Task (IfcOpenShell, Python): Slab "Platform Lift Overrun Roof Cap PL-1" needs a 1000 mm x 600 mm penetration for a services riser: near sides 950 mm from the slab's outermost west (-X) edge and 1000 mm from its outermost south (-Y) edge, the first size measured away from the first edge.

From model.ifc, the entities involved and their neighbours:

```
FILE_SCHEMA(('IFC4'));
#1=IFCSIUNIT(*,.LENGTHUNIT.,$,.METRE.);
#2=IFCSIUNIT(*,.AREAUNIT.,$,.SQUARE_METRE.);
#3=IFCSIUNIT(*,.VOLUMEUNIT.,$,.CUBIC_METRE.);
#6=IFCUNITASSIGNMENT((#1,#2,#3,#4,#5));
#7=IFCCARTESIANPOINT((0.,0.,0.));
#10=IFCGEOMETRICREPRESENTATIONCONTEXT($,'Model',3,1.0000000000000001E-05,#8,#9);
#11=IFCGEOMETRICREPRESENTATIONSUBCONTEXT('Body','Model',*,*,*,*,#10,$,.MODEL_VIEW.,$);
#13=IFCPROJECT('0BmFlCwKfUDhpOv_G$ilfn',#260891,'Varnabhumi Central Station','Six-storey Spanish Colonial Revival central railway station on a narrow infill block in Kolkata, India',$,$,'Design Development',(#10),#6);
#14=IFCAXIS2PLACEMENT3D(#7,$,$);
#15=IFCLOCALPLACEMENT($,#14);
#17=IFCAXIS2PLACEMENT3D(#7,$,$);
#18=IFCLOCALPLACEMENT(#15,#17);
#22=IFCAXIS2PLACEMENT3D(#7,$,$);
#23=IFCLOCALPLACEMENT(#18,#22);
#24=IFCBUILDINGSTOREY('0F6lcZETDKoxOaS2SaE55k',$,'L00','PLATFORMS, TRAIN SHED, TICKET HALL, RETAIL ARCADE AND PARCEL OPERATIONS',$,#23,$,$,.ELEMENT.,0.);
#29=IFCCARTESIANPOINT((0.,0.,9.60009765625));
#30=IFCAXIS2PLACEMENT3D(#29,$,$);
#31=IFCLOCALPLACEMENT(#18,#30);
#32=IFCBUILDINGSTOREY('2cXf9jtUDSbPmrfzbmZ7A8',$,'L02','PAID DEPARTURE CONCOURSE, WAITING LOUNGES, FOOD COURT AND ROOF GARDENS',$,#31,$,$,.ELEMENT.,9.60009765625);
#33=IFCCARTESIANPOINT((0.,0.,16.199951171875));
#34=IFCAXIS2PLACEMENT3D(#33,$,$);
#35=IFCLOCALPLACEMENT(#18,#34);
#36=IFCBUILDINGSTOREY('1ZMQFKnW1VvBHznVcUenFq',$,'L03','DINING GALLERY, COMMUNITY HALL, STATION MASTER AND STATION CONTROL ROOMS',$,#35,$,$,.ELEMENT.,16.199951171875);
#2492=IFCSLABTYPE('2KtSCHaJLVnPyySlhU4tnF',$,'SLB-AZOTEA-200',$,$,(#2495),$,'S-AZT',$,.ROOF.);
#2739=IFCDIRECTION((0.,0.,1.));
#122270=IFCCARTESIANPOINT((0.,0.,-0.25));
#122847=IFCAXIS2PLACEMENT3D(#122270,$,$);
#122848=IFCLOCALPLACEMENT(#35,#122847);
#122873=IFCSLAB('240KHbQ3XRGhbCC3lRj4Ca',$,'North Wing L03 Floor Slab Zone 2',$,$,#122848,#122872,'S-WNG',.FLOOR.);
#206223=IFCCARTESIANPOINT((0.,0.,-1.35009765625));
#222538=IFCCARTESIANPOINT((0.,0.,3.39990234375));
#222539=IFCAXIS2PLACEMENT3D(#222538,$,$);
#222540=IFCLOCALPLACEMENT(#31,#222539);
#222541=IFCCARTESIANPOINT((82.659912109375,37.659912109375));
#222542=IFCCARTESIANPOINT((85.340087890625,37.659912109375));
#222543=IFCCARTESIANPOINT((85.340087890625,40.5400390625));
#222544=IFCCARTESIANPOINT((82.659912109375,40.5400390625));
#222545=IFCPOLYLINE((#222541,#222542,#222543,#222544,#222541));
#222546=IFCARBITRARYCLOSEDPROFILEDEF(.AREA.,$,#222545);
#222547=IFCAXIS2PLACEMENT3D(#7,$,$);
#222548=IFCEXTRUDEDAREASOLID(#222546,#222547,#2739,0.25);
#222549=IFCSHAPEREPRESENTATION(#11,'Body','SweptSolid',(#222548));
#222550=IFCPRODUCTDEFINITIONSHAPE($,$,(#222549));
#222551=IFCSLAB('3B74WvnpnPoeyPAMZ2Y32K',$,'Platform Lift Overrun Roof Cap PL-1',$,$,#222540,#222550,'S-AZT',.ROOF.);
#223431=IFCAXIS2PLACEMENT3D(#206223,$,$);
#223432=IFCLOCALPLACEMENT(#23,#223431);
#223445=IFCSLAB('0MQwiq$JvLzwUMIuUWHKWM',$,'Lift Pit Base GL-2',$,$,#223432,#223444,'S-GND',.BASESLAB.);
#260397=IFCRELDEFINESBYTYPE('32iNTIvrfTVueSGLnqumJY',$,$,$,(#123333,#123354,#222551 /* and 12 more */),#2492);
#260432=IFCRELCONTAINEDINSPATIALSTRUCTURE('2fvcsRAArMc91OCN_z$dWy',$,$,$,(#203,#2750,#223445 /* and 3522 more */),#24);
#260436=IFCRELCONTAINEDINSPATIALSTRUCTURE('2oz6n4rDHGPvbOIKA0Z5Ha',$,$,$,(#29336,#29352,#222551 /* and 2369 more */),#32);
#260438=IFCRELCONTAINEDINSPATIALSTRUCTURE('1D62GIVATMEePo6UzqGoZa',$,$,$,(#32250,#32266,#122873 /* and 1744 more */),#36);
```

```python
import numpy as np
import ifcopenshell
import ifcopenshell.api.feature
import ifcopenshell.api.geometry
import ifcopenshell.api.root
import ifcopenshell.geom
import ifcopenshell.util.placement
import ifcopenshell.util.representation
import ifcopenshell.util.shape
import ifcopenshell.util.unit

model = ifcopenshell.open("model.ifc")
unit_scale = ifcopenshell.util.unit.calculate_unit_scale(model)
settings = ifcopenshell.geom.settings()


def volume(element):
    """Net volume in cubic metres, openings subtracted."""
    shape = ifcopenshell.geom.create_shape(settings, element)
    return ifcopenshell.util.shape.get_volume(shape.geometry)


slab = model.by_guid("3B74WvnpnPoeyPAMZ2Y32K")
before = volume(slab)

# Extent in the slab's own axes, in metres. The edges named are its -X and -Y sides.
slab_shape = ifcopenshell.geom.create_shape(settings, slab)
vertices = ifcopenshell.util.shape.get_vertices(slab_shape.geometry)
x_min, y_min, bottom = vertices.min(axis=0)
top = vertices[:, 2].max()

opening = ifcopenshell.api.root.create_entity(model, ifc_class="IfcOpeningElement", name="Services riser opening", predefined_type="OPENING")
context = ifcopenshell.util.representation.get_context(model, "Model", "Body", "MODEL_VIEW")
width, depth = 1, 0.6
outline = [(0.0, 0.0), (width, 0.0), (width, depth), (0.0, depth), (0.0, 0.0)]
# Overshoot both faces by 50 mm so the cut is clean.
shape = ifcopenshell.api.geometry.add_slab_representation(
    model, context=context, depth=top - bottom + 0.1, polyline=outline
)
ifcopenshell.api.geometry.assign_representation(model, product=opening, representation=shape)

matrix = ifcopenshell.util.placement.get_local_placement(slab.ObjectPlacement)
matrix[:, 3] = matrix @ np.append(np.array([x_min + 0.95, y_min + 1, bottom - 0.05]) / unit_scale, 1.0)
ifcopenshell.api.geometry.edit_object_placement(model, product=opening, matrix=matrix, is_si=False)
ifcopenshell.api.feature.add_feature(model, feature=opening, element=slab)

after = volume(slab)

print(f"slab volume {before:.3f} -> {after:.3f} m3")

model.write("model_rev.ifc")
```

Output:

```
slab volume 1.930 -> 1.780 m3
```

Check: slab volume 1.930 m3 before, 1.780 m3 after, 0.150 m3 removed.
